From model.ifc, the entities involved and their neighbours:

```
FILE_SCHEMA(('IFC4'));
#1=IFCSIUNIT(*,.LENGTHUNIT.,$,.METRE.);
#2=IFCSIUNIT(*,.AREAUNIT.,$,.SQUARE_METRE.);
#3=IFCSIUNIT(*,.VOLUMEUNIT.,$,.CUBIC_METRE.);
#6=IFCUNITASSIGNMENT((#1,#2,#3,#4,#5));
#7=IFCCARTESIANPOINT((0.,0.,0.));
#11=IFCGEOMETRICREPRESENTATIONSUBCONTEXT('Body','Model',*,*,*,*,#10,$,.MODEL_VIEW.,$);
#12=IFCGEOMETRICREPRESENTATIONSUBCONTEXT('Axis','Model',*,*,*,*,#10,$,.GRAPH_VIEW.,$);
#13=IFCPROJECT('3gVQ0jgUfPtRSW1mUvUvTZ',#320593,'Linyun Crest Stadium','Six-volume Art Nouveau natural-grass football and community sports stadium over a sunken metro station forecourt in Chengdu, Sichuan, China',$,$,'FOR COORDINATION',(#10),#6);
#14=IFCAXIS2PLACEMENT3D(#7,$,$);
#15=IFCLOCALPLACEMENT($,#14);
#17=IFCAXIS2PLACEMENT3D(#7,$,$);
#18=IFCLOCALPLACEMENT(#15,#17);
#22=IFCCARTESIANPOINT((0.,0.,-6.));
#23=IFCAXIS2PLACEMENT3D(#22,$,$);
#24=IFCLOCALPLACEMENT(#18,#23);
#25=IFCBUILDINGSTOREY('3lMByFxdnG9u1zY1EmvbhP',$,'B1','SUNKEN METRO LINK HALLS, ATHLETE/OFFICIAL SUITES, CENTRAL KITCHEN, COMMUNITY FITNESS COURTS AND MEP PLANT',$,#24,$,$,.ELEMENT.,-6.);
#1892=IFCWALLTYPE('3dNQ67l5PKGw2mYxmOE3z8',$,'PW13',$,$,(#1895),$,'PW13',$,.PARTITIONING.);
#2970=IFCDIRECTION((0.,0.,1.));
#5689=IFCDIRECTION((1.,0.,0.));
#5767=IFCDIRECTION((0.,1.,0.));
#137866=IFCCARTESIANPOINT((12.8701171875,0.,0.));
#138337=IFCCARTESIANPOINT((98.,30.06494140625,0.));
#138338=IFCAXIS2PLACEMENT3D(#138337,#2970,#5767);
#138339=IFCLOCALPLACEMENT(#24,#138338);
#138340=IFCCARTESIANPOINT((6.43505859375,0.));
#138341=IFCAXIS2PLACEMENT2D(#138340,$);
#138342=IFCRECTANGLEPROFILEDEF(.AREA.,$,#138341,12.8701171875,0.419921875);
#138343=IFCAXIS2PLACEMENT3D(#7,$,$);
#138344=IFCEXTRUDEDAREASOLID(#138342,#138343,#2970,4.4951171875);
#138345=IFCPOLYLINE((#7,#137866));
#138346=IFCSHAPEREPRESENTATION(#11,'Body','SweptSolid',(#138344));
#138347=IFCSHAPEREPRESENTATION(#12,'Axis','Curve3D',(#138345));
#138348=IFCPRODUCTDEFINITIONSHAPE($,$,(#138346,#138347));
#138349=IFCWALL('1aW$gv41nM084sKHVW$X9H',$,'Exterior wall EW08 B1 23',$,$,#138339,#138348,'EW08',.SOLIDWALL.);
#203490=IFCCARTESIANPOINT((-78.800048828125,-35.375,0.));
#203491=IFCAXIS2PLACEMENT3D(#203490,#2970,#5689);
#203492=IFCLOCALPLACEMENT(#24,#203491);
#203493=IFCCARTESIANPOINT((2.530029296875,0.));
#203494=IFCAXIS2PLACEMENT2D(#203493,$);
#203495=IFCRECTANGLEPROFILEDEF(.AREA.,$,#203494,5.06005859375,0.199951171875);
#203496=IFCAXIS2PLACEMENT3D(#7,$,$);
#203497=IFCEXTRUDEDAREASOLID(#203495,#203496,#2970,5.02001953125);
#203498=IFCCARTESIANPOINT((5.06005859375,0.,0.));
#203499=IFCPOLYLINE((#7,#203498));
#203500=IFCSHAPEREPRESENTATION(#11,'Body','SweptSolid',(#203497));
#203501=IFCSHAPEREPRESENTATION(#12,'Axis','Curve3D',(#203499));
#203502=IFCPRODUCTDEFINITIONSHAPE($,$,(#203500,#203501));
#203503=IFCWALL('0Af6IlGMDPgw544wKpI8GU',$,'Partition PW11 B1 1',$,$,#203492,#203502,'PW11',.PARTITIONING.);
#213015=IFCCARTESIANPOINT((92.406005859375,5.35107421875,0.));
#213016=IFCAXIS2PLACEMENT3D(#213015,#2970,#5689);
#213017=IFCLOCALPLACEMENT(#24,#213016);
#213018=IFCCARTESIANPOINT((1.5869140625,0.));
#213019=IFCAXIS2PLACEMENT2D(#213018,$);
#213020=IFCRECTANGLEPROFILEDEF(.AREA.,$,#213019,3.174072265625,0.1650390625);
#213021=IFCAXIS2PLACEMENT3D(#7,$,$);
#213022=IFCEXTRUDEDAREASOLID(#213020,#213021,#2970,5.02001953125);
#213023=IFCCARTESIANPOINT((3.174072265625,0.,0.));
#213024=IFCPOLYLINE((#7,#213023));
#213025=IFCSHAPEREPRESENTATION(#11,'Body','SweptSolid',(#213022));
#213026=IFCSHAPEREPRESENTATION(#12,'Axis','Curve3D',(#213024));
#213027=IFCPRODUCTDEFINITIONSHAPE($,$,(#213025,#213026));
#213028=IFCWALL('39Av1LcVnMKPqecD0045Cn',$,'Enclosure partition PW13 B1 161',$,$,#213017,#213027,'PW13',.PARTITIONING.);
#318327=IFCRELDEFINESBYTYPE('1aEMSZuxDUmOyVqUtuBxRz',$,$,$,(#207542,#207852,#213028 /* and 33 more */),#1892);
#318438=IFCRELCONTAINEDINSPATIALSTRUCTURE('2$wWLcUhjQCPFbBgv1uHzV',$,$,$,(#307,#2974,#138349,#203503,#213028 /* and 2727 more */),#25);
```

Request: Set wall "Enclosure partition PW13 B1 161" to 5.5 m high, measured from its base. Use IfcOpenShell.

```python
import ifcopenshell
import ifcopenshell.geom
import ifcopenshell.util.representation
import ifcopenshell.util.shape

model = ifcopenshell.open("model.ifc")
settings = ifcopenshell.geom.settings()


def volume(element):
    """Net volume in cubic metres, openings subtracted."""
    shape = ifcopenshell.geom.create_shape(settings, element)
    return ifcopenshell.util.shape.get_volume(shape.geometry)


wall = model.by_guid("39Av1LcVnMKPqecD0045Cn")
before = volume(wall)

body = ifcopenshell.util.representation.get_representation(wall, "Model", "Body")
solid = body.Items[0]
old_height = solid.Depth
solid.Depth = 5.5
after = volume(wall)

print(f"height {old_height:g} -> {solid.Depth:g}, volume {before:.3f} -> {after:.3f} m3")

model.write("model_rev.ifc")
```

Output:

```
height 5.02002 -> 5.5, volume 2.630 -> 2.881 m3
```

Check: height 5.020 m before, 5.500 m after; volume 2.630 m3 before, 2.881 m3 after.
